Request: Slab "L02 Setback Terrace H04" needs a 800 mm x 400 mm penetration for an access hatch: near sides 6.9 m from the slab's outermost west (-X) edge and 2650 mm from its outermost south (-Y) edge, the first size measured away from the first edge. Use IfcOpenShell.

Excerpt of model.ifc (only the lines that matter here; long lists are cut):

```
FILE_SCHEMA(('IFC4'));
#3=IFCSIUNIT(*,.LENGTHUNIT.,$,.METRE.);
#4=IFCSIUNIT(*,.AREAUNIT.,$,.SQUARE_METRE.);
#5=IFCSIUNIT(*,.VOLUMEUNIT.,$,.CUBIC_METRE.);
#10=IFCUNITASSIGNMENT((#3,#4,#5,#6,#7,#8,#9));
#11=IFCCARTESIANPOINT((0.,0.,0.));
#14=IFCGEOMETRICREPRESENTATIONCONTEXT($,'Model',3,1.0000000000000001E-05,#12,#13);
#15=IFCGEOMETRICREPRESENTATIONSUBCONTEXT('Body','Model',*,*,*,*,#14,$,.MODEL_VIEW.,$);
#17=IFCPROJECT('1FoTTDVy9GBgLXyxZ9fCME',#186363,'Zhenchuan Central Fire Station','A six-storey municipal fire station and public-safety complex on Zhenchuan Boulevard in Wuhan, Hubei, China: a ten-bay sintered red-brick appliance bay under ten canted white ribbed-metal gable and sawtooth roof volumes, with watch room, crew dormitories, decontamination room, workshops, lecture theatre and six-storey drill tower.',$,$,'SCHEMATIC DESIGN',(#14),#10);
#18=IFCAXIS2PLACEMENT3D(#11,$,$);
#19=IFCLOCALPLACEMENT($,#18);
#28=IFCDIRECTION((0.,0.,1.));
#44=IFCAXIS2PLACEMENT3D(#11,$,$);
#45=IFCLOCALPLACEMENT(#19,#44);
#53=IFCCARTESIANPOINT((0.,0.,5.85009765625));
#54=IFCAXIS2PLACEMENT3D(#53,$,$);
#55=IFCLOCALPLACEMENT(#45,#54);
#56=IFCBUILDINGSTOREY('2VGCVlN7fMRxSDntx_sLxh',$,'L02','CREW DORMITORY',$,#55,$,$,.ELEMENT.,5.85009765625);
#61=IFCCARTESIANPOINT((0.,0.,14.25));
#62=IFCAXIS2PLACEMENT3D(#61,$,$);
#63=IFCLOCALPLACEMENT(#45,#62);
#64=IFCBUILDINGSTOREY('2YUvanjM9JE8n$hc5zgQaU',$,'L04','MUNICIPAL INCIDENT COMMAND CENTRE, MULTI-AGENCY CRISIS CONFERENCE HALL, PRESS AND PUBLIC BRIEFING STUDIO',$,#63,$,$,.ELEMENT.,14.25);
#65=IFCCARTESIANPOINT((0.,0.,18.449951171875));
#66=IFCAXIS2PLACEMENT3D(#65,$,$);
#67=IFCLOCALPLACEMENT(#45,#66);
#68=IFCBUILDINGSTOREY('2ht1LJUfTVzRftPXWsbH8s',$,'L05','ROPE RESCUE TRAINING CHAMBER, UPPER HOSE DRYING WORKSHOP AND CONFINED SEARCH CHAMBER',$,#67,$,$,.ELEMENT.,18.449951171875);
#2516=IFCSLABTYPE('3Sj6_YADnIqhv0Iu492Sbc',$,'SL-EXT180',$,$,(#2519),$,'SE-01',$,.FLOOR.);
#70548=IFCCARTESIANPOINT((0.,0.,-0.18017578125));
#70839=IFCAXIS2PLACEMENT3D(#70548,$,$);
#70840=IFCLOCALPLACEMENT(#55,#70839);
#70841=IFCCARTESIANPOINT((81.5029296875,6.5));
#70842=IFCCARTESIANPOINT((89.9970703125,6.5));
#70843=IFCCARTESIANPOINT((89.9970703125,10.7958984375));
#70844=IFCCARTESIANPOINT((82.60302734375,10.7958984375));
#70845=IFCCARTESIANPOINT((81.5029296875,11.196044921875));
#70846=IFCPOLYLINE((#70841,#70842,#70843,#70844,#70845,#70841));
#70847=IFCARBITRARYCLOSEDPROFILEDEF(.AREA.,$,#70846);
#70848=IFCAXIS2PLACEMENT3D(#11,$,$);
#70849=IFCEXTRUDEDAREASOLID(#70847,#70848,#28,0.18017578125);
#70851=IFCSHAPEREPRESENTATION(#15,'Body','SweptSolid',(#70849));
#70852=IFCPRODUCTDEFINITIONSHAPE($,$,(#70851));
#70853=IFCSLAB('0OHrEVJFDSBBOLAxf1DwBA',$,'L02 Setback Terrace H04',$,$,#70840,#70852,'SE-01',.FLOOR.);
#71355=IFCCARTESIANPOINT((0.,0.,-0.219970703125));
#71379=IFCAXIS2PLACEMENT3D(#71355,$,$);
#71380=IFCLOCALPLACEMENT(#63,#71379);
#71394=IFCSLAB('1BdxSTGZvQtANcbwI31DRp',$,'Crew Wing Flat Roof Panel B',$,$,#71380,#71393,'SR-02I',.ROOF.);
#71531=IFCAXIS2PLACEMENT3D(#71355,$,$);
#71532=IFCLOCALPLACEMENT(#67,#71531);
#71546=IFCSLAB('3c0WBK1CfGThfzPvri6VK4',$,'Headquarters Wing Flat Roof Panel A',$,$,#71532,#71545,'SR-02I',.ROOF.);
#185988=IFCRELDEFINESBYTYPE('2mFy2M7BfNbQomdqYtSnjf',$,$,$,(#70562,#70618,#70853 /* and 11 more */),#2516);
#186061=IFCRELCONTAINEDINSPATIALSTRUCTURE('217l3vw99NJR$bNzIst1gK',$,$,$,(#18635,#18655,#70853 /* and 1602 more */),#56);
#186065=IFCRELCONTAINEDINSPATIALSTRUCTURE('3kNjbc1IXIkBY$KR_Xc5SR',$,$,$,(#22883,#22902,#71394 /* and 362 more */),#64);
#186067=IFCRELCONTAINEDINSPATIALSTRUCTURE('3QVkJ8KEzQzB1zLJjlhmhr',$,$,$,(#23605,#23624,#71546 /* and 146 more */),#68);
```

```python
import numpy as np
import ifcopenshell
import ifcopenshell.api.feature
import ifcopenshell.api.geometry
import ifcopenshell.api.root
import ifcopenshell.geom
import ifcopenshell.util.placement
import ifcopenshell.util.representation
import ifcopenshell.util.shape
import ifcopenshell.util.unit

model = ifcopenshell.open("model.ifc")
unit_scale = ifcopenshell.util.unit.calculate_unit_scale(model)
settings = ifcopenshell.geom.settings()


def volume(element):
    """Net volume in cubic metres, openings subtracted."""
    shape = ifcopenshell.geom.create_shape(settings, element)
    return ifcopenshell.util.shape.get_volume(shape.geometry)


slab = model.by_id(70853)
before = volume(slab)

# Extent in the slab's own axes, in metres. The edges named are its -X and -Y sides.
slab_shape = ifcopenshell.geom.create_shape(settings, slab)
vertices = ifcopenshell.util.shape.get_vertices(slab_shape.geometry)
x_min, y_min, bottom = vertices.min(axis=0)
top = vertices[:, 2].max()

opening = ifcopenshell.api.root.create_entity(model, ifc_class="IfcOpeningElement", name="Access hatch opening", predefined_type="OPENING")
context = ifcopenshell.util.representation.get_context(model, "Model", "Body", "MODEL_VIEW")
width, depth = 0.8, 0.4
outline = [(0.0, 0.0), (width, 0.0), (width, depth), (0.0, depth), (0.0, 0.0)]
# Overshoot both faces by 50 mm so the cut is clean.
shape = ifcopenshell.api.geometry.add_slab_representation(
    model, context=context, depth=top - bottom + 0.1, polyline=outline
)
ifcopenshell.api.geometry.assign_representation(model, product=opening, representation=shape)

matrix = ifcopenshell.util.placement.get_local_placement(slab.ObjectPlacement)
matrix[:, 3] = matrix @ np.append(np.array([x_min + 6.9, y_min + 2.65, bottom - 0.05]) / unit_scale, 1.0)
ifcopenshell.api.geometry.edit_object_placement(model, product=opening, matrix=matrix, is_si=False)
ifcopenshell.api.feature.add_feature(model, feature=opening, element=slab)

after = volume(slab)

print(f"slab volume {before:.3f} -> {after:.3f} m3")

model.write("model_updated.ifc")
```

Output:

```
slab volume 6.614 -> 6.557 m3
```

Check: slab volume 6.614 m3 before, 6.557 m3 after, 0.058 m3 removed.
